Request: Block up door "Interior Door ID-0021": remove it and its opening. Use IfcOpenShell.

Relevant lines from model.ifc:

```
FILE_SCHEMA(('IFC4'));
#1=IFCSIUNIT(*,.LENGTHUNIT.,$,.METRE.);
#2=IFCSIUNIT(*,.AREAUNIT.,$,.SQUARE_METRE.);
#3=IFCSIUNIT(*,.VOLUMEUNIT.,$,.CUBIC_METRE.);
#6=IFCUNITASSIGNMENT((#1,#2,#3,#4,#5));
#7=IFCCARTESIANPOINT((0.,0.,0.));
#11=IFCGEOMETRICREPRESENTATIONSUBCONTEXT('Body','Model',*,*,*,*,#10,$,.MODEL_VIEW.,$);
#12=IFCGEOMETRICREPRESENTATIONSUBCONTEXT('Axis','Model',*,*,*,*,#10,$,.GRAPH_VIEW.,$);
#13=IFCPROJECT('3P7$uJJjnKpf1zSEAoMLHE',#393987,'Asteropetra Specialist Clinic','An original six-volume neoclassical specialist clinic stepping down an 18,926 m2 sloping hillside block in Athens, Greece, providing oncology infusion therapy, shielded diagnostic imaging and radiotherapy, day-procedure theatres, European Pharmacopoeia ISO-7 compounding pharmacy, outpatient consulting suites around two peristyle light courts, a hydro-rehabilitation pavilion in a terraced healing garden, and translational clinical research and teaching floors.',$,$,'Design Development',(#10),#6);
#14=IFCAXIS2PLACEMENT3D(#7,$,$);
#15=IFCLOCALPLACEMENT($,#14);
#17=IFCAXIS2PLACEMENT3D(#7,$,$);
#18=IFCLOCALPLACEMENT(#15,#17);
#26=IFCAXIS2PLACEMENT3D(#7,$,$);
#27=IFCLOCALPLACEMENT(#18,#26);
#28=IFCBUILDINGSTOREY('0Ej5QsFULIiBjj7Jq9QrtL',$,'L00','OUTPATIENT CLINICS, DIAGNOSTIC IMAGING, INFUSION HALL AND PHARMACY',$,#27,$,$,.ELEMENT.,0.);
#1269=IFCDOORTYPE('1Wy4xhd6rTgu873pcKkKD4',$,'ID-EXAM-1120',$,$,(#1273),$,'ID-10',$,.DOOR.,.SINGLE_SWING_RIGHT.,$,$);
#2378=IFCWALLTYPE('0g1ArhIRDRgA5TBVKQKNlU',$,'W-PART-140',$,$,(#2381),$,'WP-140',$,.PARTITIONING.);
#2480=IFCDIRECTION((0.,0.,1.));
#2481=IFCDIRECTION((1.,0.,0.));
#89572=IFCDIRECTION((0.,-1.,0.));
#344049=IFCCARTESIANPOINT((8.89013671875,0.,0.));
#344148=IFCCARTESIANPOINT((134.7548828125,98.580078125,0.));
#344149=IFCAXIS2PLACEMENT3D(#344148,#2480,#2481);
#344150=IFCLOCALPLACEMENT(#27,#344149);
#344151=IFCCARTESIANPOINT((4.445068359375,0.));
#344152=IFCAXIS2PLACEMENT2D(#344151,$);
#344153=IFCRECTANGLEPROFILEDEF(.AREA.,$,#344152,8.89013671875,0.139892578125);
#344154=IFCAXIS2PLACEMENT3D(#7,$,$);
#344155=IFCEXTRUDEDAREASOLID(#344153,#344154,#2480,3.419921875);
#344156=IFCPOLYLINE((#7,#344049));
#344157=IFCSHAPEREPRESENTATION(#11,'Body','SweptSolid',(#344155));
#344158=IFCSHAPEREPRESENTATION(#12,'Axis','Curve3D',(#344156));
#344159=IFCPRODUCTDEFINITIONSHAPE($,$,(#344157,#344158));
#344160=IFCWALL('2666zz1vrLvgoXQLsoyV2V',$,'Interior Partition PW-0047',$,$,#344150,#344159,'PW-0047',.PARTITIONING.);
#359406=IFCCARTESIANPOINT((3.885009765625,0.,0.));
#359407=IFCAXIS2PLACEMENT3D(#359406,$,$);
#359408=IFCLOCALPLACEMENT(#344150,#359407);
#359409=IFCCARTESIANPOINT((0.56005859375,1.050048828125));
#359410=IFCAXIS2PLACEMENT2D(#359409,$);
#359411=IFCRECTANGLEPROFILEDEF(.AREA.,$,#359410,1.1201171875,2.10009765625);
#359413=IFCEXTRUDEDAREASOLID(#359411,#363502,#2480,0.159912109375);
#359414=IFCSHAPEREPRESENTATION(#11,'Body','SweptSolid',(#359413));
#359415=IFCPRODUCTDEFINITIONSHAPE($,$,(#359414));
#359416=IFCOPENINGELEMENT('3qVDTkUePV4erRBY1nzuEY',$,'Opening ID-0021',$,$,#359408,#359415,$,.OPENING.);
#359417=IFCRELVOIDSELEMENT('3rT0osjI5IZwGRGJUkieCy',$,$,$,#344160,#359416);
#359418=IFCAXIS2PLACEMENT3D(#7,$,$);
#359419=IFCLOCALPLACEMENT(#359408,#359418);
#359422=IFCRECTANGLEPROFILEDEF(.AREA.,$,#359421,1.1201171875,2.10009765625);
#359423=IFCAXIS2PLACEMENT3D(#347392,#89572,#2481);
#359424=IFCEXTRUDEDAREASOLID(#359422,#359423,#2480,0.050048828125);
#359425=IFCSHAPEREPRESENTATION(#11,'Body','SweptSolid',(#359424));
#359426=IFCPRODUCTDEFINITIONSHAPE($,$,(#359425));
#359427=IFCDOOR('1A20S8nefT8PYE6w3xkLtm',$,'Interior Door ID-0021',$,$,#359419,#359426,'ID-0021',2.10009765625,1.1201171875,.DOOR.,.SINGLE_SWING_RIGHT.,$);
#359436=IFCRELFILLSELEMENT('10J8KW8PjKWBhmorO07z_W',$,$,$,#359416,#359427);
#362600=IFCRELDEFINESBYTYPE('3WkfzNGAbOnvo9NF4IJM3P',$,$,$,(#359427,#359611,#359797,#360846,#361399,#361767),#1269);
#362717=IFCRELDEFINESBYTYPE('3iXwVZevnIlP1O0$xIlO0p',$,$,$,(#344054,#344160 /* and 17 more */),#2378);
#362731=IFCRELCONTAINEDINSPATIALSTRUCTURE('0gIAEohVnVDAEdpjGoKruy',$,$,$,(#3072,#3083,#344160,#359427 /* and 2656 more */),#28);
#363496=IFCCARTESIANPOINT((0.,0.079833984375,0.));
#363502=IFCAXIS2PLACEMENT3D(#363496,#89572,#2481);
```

```python
import ifcopenshell
import ifcopenshell.api.feature
import ifcopenshell.api.root
import ifcopenshell.geom
import ifcopenshell.util.shape

model = ifcopenshell.open("model.ifc")
settings = ifcopenshell.geom.settings()


def volume(element):
    """Net volume in cubic metres, openings subtracted."""
    shape = ifcopenshell.geom.create_shape(settings, element)
    return ifcopenshell.util.shape.get_volume(shape.geometry)


door = model.by_guid("1A20S8nefT8PYE6w3xkLtm")
opening = door.FillsVoids[0].RelatingOpeningElement
wall = opening.VoidsElements[0].RelatingBuildingElement
before = volume(wall)

ifcopenshell.api.root.remove_product(model, product=door)
ifcopenshell.api.feature.remove_feature(model, feature=opening)

after = volume(wall)

print(f"wall volume {before:.3f} -> {after:.3f} m3")

model.write("model_v2.ifc")
```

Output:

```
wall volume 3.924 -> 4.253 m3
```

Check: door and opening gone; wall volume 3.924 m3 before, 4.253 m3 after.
